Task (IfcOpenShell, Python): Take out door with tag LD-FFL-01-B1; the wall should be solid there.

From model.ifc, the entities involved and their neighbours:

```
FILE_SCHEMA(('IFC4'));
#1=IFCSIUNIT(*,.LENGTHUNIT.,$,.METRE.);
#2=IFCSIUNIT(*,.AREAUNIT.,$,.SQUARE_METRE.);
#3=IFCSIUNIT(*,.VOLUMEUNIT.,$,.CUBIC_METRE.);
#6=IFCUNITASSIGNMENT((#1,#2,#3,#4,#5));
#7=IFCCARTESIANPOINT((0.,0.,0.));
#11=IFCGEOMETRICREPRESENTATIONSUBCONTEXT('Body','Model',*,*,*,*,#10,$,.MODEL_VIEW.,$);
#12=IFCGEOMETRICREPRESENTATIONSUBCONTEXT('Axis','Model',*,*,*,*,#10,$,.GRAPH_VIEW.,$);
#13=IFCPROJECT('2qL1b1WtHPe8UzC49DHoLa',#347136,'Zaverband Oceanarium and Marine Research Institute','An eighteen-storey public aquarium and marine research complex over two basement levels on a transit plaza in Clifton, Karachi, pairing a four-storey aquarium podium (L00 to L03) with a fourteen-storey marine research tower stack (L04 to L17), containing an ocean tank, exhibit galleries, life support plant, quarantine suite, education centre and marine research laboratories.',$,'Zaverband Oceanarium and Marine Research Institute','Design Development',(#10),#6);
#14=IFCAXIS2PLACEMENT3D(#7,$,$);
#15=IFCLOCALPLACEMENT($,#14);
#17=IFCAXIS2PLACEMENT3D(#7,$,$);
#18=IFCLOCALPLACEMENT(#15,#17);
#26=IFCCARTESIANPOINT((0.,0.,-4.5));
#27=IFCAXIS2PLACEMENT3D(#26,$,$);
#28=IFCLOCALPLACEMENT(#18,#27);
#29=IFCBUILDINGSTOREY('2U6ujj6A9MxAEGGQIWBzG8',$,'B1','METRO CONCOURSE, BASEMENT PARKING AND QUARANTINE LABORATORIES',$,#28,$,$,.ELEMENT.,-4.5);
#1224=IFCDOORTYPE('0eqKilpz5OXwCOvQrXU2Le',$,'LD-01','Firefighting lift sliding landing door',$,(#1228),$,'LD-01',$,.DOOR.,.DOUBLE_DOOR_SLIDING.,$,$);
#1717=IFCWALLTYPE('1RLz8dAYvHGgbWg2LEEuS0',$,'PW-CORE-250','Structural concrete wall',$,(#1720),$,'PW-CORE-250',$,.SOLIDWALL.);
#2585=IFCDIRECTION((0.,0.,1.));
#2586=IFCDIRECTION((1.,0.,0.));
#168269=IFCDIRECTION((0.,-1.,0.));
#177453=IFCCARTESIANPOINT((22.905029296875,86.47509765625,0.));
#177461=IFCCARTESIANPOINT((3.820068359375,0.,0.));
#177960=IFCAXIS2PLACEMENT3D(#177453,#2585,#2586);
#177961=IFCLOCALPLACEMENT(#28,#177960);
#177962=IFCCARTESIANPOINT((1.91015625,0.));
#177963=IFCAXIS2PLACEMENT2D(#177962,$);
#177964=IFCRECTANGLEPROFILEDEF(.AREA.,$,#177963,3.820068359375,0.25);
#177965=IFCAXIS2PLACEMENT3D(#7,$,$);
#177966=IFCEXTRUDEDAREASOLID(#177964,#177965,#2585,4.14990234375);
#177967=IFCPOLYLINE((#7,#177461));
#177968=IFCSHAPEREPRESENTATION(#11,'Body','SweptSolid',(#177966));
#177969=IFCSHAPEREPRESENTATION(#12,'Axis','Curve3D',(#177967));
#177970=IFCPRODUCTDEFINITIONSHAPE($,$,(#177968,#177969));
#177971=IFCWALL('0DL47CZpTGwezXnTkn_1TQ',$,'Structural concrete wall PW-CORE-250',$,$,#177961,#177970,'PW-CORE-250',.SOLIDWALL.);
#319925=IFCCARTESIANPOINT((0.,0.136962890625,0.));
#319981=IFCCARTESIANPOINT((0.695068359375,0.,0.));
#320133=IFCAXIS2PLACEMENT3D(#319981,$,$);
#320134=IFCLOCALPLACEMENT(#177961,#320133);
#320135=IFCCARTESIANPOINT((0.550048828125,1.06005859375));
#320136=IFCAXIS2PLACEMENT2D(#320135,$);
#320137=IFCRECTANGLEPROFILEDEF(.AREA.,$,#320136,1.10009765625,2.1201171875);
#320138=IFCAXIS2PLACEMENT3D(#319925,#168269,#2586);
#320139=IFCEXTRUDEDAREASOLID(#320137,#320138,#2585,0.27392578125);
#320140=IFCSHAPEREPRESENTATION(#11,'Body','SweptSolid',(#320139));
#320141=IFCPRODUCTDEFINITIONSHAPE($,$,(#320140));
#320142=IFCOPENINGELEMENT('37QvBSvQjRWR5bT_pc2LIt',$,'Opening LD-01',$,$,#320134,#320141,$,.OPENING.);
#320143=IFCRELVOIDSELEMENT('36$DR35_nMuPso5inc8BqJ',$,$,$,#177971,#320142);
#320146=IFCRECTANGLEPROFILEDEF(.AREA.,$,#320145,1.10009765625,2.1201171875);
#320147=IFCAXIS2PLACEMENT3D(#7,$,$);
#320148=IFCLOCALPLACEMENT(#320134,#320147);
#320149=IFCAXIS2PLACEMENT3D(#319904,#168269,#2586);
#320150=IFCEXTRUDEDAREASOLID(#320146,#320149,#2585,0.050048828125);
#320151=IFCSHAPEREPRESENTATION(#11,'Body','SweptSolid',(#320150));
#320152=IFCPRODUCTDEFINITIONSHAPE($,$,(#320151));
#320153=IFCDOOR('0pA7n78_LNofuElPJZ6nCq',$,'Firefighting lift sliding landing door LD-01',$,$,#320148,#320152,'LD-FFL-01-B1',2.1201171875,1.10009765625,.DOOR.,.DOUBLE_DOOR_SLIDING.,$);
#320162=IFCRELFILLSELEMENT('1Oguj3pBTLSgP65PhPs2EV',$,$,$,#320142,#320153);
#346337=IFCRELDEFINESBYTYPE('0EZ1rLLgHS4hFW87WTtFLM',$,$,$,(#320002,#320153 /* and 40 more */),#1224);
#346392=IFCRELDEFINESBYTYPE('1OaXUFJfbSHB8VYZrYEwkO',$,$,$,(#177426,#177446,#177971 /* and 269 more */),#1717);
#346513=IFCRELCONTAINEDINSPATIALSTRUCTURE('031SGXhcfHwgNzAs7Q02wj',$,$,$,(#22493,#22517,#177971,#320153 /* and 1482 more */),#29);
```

```python
import ifcopenshell
import ifcopenshell.api.feature
import ifcopenshell.api.root
import ifcopenshell.geom
import ifcopenshell.util.shape

model = ifcopenshell.open("model.ifc")
settings = ifcopenshell.geom.settings()


def volume(element):
    """Net volume in cubic metres, openings subtracted."""
    shape = ifcopenshell.geom.create_shape(settings, element)
    return ifcopenshell.util.shape.get_volume(shape.geometry)


door = model.by_guid("0pA7n78_LNofuElPJZ6nCq")
opening = door.FillsVoids[0].RelatingOpeningElement
wall = opening.VoidsElements[0].RelatingBuildingElement
before = volume(wall)

ifcopenshell.api.root.remove_product(model, product=door)
ifcopenshell.api.feature.remove_feature(model, feature=opening)

after = volume(wall)

print(f"wall volume {before:.3f} -> {after:.3f} m3")

model.write("model_rev.ifc")
```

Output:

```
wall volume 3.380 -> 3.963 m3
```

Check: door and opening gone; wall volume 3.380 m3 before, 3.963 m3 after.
